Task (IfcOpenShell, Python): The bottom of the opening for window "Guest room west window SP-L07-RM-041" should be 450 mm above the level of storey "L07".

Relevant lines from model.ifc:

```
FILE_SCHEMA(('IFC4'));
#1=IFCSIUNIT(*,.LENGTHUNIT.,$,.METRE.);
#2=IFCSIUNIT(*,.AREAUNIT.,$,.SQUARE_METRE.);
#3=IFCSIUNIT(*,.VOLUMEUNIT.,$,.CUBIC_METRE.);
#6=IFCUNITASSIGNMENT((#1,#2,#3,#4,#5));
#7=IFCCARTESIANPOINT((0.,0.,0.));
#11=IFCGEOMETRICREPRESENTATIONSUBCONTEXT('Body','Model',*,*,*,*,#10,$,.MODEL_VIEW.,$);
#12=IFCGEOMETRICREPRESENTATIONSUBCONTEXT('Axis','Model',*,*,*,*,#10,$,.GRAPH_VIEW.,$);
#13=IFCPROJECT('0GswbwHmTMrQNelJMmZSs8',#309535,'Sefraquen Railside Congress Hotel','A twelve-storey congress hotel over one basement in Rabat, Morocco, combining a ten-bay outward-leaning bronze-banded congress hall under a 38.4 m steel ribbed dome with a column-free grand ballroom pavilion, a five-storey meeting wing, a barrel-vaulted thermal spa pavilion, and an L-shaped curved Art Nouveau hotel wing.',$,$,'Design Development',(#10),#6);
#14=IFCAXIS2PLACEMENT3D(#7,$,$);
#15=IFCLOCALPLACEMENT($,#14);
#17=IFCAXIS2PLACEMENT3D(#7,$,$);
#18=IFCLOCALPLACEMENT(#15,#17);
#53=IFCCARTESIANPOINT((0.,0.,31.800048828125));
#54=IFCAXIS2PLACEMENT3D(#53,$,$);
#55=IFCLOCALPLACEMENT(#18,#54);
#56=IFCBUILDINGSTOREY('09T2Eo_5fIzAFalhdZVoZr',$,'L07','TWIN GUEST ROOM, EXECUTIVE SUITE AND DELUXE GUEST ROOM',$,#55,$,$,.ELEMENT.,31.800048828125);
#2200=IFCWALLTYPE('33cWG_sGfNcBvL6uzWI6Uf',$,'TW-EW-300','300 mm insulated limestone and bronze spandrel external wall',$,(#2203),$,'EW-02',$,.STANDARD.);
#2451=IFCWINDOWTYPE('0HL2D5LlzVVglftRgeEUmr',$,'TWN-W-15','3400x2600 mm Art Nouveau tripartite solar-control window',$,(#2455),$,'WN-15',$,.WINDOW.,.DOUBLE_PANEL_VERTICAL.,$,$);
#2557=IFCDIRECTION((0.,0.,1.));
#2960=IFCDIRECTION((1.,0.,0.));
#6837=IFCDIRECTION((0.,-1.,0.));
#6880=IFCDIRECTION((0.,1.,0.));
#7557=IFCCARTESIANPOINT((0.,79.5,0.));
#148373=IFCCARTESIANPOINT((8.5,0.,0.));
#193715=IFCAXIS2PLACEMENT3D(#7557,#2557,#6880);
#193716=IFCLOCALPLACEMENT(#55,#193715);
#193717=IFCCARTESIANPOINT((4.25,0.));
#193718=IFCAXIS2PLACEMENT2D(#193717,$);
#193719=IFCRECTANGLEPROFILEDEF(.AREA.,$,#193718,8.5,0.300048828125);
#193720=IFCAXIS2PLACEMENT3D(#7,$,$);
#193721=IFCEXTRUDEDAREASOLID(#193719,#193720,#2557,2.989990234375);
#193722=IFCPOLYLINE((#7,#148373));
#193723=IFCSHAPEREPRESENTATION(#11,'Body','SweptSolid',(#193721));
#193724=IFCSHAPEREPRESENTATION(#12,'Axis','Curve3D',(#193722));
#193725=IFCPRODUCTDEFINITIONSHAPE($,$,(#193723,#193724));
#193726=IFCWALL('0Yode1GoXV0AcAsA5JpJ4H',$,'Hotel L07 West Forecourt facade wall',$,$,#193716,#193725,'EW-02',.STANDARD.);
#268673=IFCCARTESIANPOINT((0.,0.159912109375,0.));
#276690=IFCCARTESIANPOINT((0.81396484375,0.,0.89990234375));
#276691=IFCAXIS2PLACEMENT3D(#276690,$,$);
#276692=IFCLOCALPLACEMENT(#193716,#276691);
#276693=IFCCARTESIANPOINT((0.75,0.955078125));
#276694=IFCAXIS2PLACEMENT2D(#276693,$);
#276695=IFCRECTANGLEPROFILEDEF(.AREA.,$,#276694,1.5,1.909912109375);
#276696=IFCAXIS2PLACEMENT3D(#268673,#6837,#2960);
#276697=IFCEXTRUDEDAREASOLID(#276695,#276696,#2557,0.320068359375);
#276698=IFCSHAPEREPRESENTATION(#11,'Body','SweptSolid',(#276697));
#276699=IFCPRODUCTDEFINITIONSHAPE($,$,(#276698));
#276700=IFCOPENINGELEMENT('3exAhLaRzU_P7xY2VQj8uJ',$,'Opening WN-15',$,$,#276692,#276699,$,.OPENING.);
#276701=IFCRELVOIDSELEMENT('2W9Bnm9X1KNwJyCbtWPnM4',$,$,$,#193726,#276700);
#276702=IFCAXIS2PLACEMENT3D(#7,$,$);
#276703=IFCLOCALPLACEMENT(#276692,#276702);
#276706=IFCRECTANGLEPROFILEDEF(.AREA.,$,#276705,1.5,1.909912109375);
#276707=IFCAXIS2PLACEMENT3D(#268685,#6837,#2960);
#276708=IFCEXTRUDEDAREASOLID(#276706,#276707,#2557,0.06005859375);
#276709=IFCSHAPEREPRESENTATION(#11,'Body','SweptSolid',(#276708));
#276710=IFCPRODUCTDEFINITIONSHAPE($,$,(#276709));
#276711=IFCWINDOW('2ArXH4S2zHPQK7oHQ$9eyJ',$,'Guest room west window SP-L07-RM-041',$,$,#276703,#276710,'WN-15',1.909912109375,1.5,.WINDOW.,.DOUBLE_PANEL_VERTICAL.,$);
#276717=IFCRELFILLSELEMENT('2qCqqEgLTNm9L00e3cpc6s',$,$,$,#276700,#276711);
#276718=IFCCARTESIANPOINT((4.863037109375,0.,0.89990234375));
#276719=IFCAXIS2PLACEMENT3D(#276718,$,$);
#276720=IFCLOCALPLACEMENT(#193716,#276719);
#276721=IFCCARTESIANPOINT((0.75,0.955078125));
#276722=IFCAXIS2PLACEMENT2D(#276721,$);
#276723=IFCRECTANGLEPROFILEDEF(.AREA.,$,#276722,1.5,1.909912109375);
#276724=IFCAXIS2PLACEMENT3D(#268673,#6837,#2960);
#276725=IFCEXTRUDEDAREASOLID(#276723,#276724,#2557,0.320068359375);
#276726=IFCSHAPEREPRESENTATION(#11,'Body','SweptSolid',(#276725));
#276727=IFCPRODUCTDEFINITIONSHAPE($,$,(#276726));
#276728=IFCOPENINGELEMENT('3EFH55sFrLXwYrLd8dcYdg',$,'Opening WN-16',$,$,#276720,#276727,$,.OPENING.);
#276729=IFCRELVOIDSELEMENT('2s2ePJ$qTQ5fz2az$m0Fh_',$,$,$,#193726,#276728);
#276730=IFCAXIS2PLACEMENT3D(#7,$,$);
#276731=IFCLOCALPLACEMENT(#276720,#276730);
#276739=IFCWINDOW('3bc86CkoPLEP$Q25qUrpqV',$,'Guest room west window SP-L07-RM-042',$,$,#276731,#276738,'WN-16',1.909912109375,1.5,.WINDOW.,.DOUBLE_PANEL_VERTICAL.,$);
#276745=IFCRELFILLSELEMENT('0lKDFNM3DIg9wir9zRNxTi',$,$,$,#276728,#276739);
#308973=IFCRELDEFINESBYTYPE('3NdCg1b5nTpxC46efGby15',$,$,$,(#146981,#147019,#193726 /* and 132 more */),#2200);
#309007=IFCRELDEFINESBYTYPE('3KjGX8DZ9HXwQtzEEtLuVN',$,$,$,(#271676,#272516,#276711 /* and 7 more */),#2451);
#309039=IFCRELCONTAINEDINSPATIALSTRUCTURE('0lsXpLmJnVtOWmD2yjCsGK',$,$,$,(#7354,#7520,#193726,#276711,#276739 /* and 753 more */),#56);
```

```python
import numpy as np
import ifcopenshell
import ifcopenshell.api.geometry
import ifcopenshell.geom
import ifcopenshell.util.element
import ifcopenshell.util.placement
import ifcopenshell.util.shape
import ifcopenshell.util.unit

model = ifcopenshell.open("model.ifc")
unit_scale = ifcopenshell.util.unit.calculate_unit_scale(model)

window = model.by_id(276711)
opening = window.FillsVoids[0].RelatingOpeningElement
storey = ifcopenshell.util.element.get_container(window, ifc_class="IfcBuildingStorey")
level = ifcopenshell.util.placement.get_local_placement(storey.ObjectPlacement)[2, 3]

# The opening's origin need not be at the sill, so measure its lowest point.
shape = ifcopenshell.geom.create_shape(ifcopenshell.geom.settings(), opening)
bottom = ifcopenshell.util.shape.get_shape_bottom_elevation(shape, shape.geometry) / unit_scale
dz = level + 0.45 / unit_scale - bottom

shift = np.array([0.0, 0.0, dz])
# The window is placed relative to its opening, so it follows when the opening moves.
matrix = ifcopenshell.util.placement.get_local_placement(opening.ObjectPlacement)
matrix[:3, 3] += shift
ifcopenshell.api.geometry.edit_object_placement(
    model, product=opening, matrix=matrix, is_si=False, should_transform_children=True
)

print(f"moved by {dz * unit_scale:+.3f} m")

model.write("model_updated.ifc")
```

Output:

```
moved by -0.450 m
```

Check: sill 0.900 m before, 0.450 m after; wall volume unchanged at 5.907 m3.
